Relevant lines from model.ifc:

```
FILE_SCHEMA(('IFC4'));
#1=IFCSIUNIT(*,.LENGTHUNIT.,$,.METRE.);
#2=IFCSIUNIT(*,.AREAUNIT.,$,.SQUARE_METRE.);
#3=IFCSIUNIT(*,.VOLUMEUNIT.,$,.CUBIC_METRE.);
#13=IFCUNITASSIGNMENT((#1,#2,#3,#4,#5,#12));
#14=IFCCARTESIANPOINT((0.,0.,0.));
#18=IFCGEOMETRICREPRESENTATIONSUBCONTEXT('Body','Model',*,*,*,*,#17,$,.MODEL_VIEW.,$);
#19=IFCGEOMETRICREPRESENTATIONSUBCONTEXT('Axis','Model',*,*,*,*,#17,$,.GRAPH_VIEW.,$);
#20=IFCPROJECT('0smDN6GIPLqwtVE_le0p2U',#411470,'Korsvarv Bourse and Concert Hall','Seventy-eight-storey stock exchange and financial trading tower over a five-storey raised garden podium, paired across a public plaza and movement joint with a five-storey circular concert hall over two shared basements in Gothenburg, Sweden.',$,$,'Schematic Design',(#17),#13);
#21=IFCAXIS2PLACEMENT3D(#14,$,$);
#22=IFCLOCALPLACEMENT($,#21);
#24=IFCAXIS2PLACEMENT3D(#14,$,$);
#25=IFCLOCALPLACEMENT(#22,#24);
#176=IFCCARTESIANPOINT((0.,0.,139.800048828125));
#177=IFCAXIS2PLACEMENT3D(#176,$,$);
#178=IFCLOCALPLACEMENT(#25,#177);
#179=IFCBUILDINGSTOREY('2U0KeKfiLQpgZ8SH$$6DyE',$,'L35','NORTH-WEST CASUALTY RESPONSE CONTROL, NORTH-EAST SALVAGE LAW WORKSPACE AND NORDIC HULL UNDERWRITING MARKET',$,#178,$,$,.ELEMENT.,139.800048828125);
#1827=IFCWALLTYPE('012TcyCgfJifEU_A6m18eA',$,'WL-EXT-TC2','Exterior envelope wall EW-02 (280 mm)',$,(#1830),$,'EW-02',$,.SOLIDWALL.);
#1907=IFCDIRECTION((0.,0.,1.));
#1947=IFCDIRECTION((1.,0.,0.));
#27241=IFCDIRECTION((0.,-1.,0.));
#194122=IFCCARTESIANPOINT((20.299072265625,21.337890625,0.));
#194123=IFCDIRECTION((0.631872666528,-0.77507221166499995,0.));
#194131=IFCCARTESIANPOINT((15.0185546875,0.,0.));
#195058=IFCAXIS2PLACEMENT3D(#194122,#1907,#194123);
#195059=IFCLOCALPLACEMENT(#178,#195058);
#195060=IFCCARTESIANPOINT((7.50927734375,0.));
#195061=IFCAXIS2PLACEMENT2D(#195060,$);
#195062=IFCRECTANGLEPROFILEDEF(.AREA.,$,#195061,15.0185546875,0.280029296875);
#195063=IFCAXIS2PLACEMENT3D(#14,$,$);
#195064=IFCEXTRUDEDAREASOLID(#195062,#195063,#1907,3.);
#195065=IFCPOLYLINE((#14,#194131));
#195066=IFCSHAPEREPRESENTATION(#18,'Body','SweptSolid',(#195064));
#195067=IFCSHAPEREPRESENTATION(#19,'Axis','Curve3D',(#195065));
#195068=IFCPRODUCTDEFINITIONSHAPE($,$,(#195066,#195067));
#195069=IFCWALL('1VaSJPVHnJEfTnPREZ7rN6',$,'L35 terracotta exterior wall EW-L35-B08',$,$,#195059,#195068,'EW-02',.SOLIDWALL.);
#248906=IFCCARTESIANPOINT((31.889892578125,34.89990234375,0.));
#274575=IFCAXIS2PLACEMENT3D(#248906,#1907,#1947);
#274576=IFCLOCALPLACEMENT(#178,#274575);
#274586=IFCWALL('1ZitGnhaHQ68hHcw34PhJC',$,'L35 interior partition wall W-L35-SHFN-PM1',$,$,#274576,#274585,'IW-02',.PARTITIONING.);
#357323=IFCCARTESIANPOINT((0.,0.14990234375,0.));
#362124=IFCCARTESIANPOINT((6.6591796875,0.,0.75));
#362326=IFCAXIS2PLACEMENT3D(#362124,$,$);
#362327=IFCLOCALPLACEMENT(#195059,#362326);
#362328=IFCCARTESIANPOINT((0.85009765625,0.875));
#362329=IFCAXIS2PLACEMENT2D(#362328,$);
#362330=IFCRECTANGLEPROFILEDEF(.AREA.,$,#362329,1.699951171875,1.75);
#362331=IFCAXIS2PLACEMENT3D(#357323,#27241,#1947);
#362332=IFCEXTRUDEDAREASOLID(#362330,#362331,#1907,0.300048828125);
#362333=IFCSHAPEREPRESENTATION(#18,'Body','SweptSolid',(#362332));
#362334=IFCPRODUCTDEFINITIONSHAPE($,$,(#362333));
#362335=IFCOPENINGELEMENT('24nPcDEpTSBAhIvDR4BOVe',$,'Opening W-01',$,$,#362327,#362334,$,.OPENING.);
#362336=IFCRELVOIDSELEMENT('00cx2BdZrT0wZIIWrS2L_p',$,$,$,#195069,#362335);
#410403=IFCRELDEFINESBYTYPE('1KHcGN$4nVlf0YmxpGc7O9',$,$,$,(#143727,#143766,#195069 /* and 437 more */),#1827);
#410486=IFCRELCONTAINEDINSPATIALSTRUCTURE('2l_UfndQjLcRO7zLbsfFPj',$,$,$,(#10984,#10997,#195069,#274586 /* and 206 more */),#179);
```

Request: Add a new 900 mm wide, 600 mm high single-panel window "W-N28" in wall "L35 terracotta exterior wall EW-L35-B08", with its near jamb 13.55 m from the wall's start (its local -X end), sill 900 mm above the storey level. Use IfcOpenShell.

```python
import numpy as np
import ifcopenshell
import ifcopenshell.api.feature
import ifcopenshell.api.geometry
import ifcopenshell.api.root
import ifcopenshell.api.spatial
import ifcopenshell.geom
import ifcopenshell.util.element
import ifcopenshell.util.placement
import ifcopenshell.util.representation
import ifcopenshell.util.shape
import ifcopenshell.util.unit

model = ifcopenshell.open("model.ifc")
unit_scale = ifcopenshell.util.unit.calculate_unit_scale(model)
settings = ifcopenshell.geom.settings()


def volume(element):
    """Net volume in cubic metres, openings subtracted."""
    shape = ifcopenshell.geom.create_shape(settings, element)
    return ifcopenshell.util.shape.get_volume(shape.geometry)


wall = model.by_guid("1VaSJPVHnJEfTnPREZ7rN6")
storey = ifcopenshell.util.element.get_container(wall, ifc_class="IfcBuildingStorey")
context = ifcopenshell.util.representation.get_context(model, "Model", "Body", "MODEL_VIEW")
before = volume(wall)

width, height, from_end, sill = 0.9, 0.6, 13.55, 0.9  # metres

# The wall runs along its own X axis, and the end named is its -X end.
wall_shape = ifcopenshell.geom.create_shape(settings, wall)
x, y, z = ifcopenshell.util.shape.get_vertices(wall_shape.geometry).T
start = x.min() + from_end
face, thickness = float(y.min()), float(y.max() - y.min())
wall_matrix = ifcopenshell.util.placement.get_local_placement(wall.ObjectPlacement)
level = ifcopenshell.util.placement.get_local_placement(storey.ObjectPlacement)[2, 3]


def in_wall(x, y):
    """Placement at x, y metres in the wall's axes, at sill height."""
    matrix = wall_matrix.copy()
    matrix[:, 3] = wall_matrix @ np.array([x / unit_scale, y / unit_scale, 0.0, 1.0])
    matrix[2, 3] = level + sill / unit_scale
    return matrix


# Opening: a box that overshoots both wall faces by 50 mm.
opening = ifcopenshell.api.root.create_entity(model, ifc_class="IfcOpeningElement", predefined_type="OPENING")
box = ifcopenshell.api.geometry.add_wall_representation(
    model, context=context, length=width, height=height, thickness=thickness + 0.1
)
ifcopenshell.api.geometry.assign_representation(model, product=opening, representation=box)
ifcopenshell.api.geometry.edit_object_placement(model, product=opening, matrix=in_wall(start, face - 0.05), is_si=False)
ifcopenshell.api.feature.add_feature(model, feature=opening, element=wall)

window = ifcopenshell.api.root.create_entity(model, ifc_class="IfcWindow", name="W-N28", predefined_type="WINDOW")
window.OverallWidth, window.OverallHeight = width / unit_scale, height / unit_scale
window.PartitioningType = "SINGLE_PANEL"
body = ifcopenshell.api.geometry.add_window_representation(
    model,
    context=context,
    overall_width=window.OverallWidth,
    overall_height=window.OverallHeight,
    partition_type="SINGLE_PANEL",
)
ifcopenshell.api.geometry.assign_representation(model, product=window, representation=body)
ifcopenshell.api.spatial.assign_container(model, products=[window], relating_structure=storey)
ifcopenshell.api.feature.add_filling(model, opening=opening, element=window)

# Centre the window in the wall's thickness.
ifcopenshell.api.geometry.edit_object_placement(model, product=window, matrix=in_wall(start, face), is_si=False)
window_shape = ifcopenshell.geom.create_shape(settings, window)
depth = ifcopenshell.util.shape.get_vertices(window_shape.geometry)[:, 1]
offset = face + thickness / 2 - (depth.min() + depth.max()) / 2
ifcopenshell.api.geometry.edit_object_placement(model, product=window, matrix=in_wall(start, offset), is_si=False)

after = volume(wall)

print(f"wall volume {before:.3f} -> {after:.3f} m3")

model.write("model_updated.ifc")
```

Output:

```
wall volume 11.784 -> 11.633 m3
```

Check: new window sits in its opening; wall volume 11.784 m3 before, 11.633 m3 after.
